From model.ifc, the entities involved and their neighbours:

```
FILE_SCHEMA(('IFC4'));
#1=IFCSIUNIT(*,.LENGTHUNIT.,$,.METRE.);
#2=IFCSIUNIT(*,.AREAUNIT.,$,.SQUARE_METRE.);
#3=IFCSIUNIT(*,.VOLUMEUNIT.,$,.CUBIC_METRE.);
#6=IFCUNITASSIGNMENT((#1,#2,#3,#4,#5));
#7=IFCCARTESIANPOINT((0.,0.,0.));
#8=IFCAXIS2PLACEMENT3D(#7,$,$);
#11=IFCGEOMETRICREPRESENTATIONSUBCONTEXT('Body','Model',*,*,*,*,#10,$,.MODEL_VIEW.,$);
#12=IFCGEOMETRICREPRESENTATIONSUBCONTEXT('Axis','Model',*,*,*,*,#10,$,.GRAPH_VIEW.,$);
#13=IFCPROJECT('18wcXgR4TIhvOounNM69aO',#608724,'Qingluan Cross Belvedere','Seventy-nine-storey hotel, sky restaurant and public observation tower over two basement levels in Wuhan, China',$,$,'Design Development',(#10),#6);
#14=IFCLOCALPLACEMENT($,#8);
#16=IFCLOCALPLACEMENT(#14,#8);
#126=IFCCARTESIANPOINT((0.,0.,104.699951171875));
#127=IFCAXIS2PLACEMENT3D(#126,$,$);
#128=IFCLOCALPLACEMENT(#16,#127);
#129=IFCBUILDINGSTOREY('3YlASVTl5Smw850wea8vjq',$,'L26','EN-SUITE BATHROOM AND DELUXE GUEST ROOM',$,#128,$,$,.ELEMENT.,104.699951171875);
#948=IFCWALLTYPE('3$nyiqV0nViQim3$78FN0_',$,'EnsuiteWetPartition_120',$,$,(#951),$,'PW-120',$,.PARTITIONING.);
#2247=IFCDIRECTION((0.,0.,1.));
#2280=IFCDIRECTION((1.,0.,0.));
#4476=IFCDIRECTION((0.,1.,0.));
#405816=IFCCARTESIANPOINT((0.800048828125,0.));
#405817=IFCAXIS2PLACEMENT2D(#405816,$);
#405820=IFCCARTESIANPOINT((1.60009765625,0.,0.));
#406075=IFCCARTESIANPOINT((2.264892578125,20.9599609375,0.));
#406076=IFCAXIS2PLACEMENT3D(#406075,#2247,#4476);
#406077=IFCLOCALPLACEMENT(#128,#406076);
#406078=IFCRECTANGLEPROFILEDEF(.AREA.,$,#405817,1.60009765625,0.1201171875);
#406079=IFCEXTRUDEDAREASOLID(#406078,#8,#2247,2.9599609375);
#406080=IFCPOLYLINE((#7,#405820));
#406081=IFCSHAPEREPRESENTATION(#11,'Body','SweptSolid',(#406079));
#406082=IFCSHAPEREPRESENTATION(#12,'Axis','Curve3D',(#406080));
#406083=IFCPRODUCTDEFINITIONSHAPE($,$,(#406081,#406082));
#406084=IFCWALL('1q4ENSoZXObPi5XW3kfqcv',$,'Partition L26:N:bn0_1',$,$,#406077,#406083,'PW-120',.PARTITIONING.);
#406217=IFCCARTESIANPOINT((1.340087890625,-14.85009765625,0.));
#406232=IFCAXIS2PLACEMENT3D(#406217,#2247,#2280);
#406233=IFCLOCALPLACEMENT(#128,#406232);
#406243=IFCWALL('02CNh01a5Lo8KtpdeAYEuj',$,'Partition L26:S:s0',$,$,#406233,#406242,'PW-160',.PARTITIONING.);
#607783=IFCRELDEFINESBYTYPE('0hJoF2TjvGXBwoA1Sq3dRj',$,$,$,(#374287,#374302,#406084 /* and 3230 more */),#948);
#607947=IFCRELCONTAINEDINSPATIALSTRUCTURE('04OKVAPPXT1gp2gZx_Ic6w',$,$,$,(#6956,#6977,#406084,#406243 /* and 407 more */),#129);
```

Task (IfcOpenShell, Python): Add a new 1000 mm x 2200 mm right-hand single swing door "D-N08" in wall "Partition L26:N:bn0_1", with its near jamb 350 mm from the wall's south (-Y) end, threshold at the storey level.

```python
import numpy as np
import ifcopenshell
import ifcopenshell.api.feature
import ifcopenshell.api.geometry
import ifcopenshell.api.root
import ifcopenshell.api.spatial
import ifcopenshell.geom
import ifcopenshell.util.element
import ifcopenshell.util.placement
import ifcopenshell.util.representation
import ifcopenshell.util.shape
import ifcopenshell.util.unit

model = ifcopenshell.open("model.ifc")
unit_scale = ifcopenshell.util.unit.calculate_unit_scale(model)
settings = ifcopenshell.geom.settings()


def volume(element):
    """Net volume in cubic metres, openings subtracted."""
    shape = ifcopenshell.geom.create_shape(settings, element)
    return ifcopenshell.util.shape.get_volume(shape.geometry)


wall = model.by_guid("1q4ENSoZXObPi5XW3kfqcv")
storey = ifcopenshell.util.element.get_container(wall, ifc_class="IfcBuildingStorey")
context = ifcopenshell.util.representation.get_context(model, "Model", "Body", "MODEL_VIEW")
before = volume(wall)

width, height, from_end, sill = 1, 2.2, 0.35, 0.0  # metres

# The wall runs along its own X axis, and the end named is its -X end.
wall_shape = ifcopenshell.geom.create_shape(settings, wall)
x, y, z = ifcopenshell.util.shape.get_vertices(wall_shape.geometry).T
start = x.min() + from_end
face, thickness = float(y.min()), float(y.max() - y.min())
wall_matrix = ifcopenshell.util.placement.get_local_placement(wall.ObjectPlacement)
level = ifcopenshell.util.placement.get_local_placement(storey.ObjectPlacement)[2, 3]


def in_wall(x, y):
    """Placement at x, y metres in the wall's axes, at sill height."""
    matrix = wall_matrix.copy()
    matrix[:, 3] = wall_matrix @ np.array([x / unit_scale, y / unit_scale, 0.0, 1.0])
    matrix[2, 3] = level + sill / unit_scale
    return matrix


# Opening: a box that overshoots both wall faces by 50 mm.
opening = ifcopenshell.api.root.create_entity(model, ifc_class="IfcOpeningElement", predefined_type="OPENING")
box = ifcopenshell.api.geometry.add_wall_representation(
    model, context=context, length=width, height=height, thickness=thickness + 0.1
)
ifcopenshell.api.geometry.assign_representation(model, product=opening, representation=box)
ifcopenshell.api.geometry.edit_object_placement(model, product=opening, matrix=in_wall(start, face - 0.05), is_si=False)
ifcopenshell.api.feature.add_feature(model, feature=opening, element=wall)

door = ifcopenshell.api.root.create_entity(model, ifc_class="IfcDoor", name="D-N08", predefined_type="DOOR")
door.OverallWidth, door.OverallHeight = width / unit_scale, height / unit_scale
door.OperationType = "SINGLE_SWING_RIGHT"
body = ifcopenshell.api.geometry.add_door_representation(
    model,
    context=context,
    overall_width=door.OverallWidth,
    overall_height=door.OverallHeight,
    operation_type="SINGLE_SWING_RIGHT",
    lining_properties={"LiningDepth": thickness / unit_scale, "ThresholdDepth": thickness / unit_scale},
)
ifcopenshell.api.geometry.assign_representation(model, product=door, representation=body)
ifcopenshell.api.spatial.assign_container(model, products=[door], relating_structure=storey)
ifcopenshell.api.feature.add_filling(model, opening=opening, element=door)

# The lining spans the wall, so the door starts at the wall face.
ifcopenshell.api.geometry.edit_object_placement(model, product=door, matrix=in_wall(start, face), is_si=False)

after = volume(wall)

print(f"wall volume {before:.3f} -> {after:.3f} m3")

model.write("model_v2.ifc")
```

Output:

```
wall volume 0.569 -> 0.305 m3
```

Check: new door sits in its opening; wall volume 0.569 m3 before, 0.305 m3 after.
